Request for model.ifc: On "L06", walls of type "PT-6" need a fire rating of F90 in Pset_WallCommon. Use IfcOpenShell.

First a look at what the model holds.

```python
import ifcopenshell
import ifcopenshell.util.element

model = ifcopenshell.open("model.ifc")
print(model.schema)
storey = next(s for s in model.by_type("IfcBuildingStorey") if s.Name == "L06")
walls = [e for e in ifcopenshell.util.element.get_decomposition(storey) if e.is_a("IfcWall")]
seen = {}
for e in walls:
    element_type = ifcopenshell.util.element.get_type(e)
    key = (element_type.Name if element_type != e and element_type else None, ifcopenshell.util.element.get_pset(e, "Pset_WallCommon", "FireRating"))
    seen[key] = seen.get(key, 0) + 1
for (name, value), count in sorted(seen.items(), key=str):
    print(count, "x", name, "|", value)
```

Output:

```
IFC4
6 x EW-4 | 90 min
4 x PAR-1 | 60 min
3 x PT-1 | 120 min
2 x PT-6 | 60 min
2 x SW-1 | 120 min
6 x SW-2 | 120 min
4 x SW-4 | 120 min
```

```python
import ifcopenshell
import ifcopenshell.api.pset
import ifcopenshell.util.element

model = ifcopenshell.open("model.ifc")

storey = next(s for s in model.by_type("IfcBuildingStorey") if s.Name == "L06")
walls = [e for e in ifcopenshell.util.element.get_decomposition(storey) if e.is_a("IfcWall")]

count = 0
for e in walls:
    element_type = ifcopenshell.util.element.get_type(e)
    if element_type in (None, e) or element_type.Name != "PT-6":
        continue
    # add_pset returns the element's existing set when there is one.
    pset = ifcopenshell.api.pset.add_pset(model, product=e, name="Pset_WallCommon")
    ifcopenshell.api.pset.edit_pset(model, pset=pset, properties={"FireRating": "F90"})
    count += 1

print(count, "walls updated")

model.write("model_edited.ifc")
```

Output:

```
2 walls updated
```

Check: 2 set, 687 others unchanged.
